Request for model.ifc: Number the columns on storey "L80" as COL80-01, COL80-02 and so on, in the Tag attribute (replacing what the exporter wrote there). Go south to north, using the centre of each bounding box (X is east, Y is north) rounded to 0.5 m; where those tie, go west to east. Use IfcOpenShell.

First a look at what the model holds.

```python
import ifcopenshell
import ifcopenshell.util.element
import ifcopenshell.util.placement

model = ifcopenshell.open("model.ifc")
print(model.schema)
storey = next(s for s in model.by_type("IfcBuildingStorey") if s.Name == "L80")
columns = [e for e in ifcopenshell.util.element.get_decomposition(storey) if e.is_a("IfcColumn")]
for e in sorted(columns, key=lambda e: e.id()):
    origin = ifcopenshell.util.placement.get_local_placement(e.ObjectPlacement)[:3, 3]
    print(e.id(), e.Tag, e.Name, origin.round(2) + 0.0, sep=" | ")
```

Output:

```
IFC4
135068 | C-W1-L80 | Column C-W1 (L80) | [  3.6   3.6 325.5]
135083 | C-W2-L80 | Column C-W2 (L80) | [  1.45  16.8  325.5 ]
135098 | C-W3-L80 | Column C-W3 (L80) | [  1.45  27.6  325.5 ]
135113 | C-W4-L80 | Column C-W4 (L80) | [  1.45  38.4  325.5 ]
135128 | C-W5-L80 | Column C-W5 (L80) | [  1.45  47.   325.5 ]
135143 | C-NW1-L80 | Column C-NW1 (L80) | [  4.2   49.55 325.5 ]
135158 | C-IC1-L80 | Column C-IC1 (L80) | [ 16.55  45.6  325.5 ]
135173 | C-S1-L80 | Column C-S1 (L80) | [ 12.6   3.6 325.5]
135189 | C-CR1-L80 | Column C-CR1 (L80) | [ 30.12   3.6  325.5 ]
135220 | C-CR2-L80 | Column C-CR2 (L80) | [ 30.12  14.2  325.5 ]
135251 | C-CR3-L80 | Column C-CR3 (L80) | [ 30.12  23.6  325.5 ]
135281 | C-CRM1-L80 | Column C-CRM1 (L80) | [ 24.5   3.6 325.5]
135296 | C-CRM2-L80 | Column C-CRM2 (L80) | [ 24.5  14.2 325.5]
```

```python
import ifcopenshell
import ifcopenshell.geom
import ifcopenshell.util.element
import ifcopenshell.util.shape

model = ifcopenshell.open("model.ifc")
settings = ifcopenshell.geom.settings()
settings.set("use-world-coords", True)


def centre(element):
    shape = ifcopenshell.geom.create_shape(settings, element)
    return ifcopenshell.util.shape.get_bbox_centroid(shape.geometry)


storey = next(s for s in model.by_type("IfcBuildingStorey") if s.Name == "L80")
columns = [e for e in ifcopenshell.util.element.get_decomposition(storey) if e.is_a("IfcColumn")]

# Insertion points can sit at a corner or the storey origin, so sort by the geometry (in metres).
centres = {e: centre(e) for e in columns}
columns.sort(key=lambda e: (round(centres[e][1] / 0.5), centres[e][0]))

for i, e in enumerate(columns, start=1):
    number = f"COL80-{i:02d}"
    e.Tag = number
    print(e.id(), number)

model.write("model_edited.ifc")
```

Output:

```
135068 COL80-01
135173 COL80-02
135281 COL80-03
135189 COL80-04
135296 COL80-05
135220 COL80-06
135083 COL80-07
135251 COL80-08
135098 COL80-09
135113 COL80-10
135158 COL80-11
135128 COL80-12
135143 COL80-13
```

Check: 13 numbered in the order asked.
